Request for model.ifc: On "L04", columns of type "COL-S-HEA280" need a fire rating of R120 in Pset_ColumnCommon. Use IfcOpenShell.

First a look at what the model holds.

```python
import ifcopenshell
import ifcopenshell.util.element

model = ifcopenshell.open("model.ifc")
print(model.schema)
storey = next(s for s in model.by_type("IfcBuildingStorey") if s.Name == "L04")
columns = [e for e in ifcopenshell.util.element.get_decomposition(storey) if e.is_a("IfcColumn")]
seen = {}
for e in columns:
    element_type = ifcopenshell.util.element.get_type(e)
    key = (element_type.Name if element_type != e and element_type else None, ifcopenshell.util.element.get_pset(e, "Pset_ColumnCommon", "FireRating"))
    seen[key] = seen.get(key, 0) + 1
for (name, value), count in sorted(seen.items(), key=str):
    print(count, "x", name, "|", value)
```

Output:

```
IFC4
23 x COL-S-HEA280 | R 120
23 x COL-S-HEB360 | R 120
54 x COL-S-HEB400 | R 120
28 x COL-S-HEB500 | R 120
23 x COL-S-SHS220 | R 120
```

```python
import ifcopenshell
import ifcopenshell.api.pset
import ifcopenshell.util.element

model = ifcopenshell.open("model.ifc")

storey = next(s for s in model.by_type("IfcBuildingStorey") if s.Name == "L04")
columns = [e for e in ifcopenshell.util.element.get_decomposition(storey) if e.is_a("IfcColumn")]

count = 0
for e in columns:
    element_type = ifcopenshell.util.element.get_type(e)
    if element_type in (None, e) or element_type.Name != "COL-S-HEA280":
        continue
    # add_pset returns the element's existing set when there is one.
    pset = ifcopenshell.api.pset.add_pset(model, product=e, name="Pset_ColumnCommon")
    ifcopenshell.api.pset.edit_pset(model, pset=pset, properties={"FireRating": "R120"})
    count += 1

print(count, "columns updated")

model.write("model_updated.ifc")
```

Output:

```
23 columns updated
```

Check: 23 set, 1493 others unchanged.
